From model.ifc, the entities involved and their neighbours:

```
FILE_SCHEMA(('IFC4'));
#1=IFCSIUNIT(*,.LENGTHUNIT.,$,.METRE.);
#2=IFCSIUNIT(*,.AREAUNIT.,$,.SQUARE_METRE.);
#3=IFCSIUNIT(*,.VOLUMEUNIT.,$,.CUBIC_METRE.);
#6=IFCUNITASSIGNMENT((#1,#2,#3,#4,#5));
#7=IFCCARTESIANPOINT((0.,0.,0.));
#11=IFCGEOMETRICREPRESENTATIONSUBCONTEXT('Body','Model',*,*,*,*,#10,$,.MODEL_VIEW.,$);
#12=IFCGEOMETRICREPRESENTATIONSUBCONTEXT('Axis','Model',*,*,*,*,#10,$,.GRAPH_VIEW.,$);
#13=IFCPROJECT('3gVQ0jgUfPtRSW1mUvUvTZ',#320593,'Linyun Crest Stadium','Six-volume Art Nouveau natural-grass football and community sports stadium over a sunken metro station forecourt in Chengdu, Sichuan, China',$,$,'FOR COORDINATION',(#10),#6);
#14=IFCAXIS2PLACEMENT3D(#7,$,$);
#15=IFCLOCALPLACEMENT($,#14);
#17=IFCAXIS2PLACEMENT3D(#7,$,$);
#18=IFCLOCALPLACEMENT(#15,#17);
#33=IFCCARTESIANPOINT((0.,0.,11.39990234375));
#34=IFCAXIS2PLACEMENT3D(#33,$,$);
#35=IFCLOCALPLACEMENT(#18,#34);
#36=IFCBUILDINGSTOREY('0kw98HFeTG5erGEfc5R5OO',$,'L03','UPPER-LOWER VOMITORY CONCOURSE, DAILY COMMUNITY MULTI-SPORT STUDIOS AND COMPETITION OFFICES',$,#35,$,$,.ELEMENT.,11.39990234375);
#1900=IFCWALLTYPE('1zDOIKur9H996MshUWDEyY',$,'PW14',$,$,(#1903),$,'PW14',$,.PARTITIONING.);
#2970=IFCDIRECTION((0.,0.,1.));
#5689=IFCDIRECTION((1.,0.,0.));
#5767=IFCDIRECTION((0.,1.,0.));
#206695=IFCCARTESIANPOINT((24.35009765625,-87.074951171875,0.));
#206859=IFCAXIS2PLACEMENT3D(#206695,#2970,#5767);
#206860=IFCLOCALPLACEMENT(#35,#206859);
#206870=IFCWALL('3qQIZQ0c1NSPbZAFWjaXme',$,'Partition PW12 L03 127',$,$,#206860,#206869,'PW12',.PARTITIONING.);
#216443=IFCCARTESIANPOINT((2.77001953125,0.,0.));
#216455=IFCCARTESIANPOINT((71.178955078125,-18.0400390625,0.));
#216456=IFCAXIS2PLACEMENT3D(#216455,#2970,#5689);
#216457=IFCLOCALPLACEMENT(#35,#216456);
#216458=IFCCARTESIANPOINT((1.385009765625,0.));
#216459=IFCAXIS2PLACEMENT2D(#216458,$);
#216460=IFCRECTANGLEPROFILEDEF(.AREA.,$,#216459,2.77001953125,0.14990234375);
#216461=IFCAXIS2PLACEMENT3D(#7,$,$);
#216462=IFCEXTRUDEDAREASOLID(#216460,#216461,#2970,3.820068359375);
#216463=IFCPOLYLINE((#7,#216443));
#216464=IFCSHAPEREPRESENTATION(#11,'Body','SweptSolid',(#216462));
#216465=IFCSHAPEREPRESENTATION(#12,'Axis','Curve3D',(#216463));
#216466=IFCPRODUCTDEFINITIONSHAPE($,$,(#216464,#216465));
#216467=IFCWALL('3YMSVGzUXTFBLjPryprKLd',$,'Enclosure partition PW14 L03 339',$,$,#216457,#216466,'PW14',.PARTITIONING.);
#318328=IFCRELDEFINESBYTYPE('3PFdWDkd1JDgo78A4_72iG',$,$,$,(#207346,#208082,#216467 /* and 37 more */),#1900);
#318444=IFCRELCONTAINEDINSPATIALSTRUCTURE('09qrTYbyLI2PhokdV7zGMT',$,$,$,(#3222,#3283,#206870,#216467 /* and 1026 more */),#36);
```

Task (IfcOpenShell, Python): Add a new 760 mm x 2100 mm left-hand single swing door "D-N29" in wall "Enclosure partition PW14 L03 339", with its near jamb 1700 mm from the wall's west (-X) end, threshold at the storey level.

```python
import numpy as np
import ifcopenshell
import ifcopenshell.api.feature
import ifcopenshell.api.geometry
import ifcopenshell.api.root
import ifcopenshell.api.spatial
import ifcopenshell.geom
import ifcopenshell.util.element
import ifcopenshell.util.placement
import ifcopenshell.util.representation
import ifcopenshell.util.shape
import ifcopenshell.util.unit

model = ifcopenshell.open("model.ifc")
unit_scale = ifcopenshell.util.unit.calculate_unit_scale(model)
settings = ifcopenshell.geom.settings()


def volume(element):
    """Net volume in cubic metres, openings subtracted."""
    shape = ifcopenshell.geom.create_shape(settings, element)
    return ifcopenshell.util.shape.get_volume(shape.geometry)


wall = model.by_guid("3YMSVGzUXTFBLjPryprKLd")
storey = ifcopenshell.util.element.get_container(wall, ifc_class="IfcBuildingStorey")
context = ifcopenshell.util.representation.get_context(model, "Model", "Body", "MODEL_VIEW")
before = volume(wall)

width, height, from_end, sill = 0.76, 2.1, 1.7, 0.0  # metres

# The wall runs along its own X axis, and the end named is its -X end.
wall_shape = ifcopenshell.geom.create_shape(settings, wall)
x, y, z = ifcopenshell.util.shape.get_vertices(wall_shape.geometry).T
start = x.min() + from_end
face, thickness = float(y.min()), float(y.max() - y.min())
wall_matrix = ifcopenshell.util.placement.get_local_placement(wall.ObjectPlacement)
level = ifcopenshell.util.placement.get_local_placement(storey.ObjectPlacement)[2, 3]


def in_wall(x, y):
    """Placement at x, y metres in the wall's axes, at sill height."""
    matrix = wall_matrix.copy()
    matrix[:, 3] = wall_matrix @ np.array([x / unit_scale, y / unit_scale, 0.0, 1.0])
    matrix[2, 3] = level + sill / unit_scale
    return matrix


# Opening: a box that overshoots both wall faces by 50 mm.
opening = ifcopenshell.api.root.create_entity(model, ifc_class="IfcOpeningElement", predefined_type="OPENING")
box = ifcopenshell.api.geometry.add_wall_representation(
    model, context=context, length=width, height=height, thickness=thickness + 0.1
)
ifcopenshell.api.geometry.assign_representation(model, product=opening, representation=box)
ifcopenshell.api.geometry.edit_object_placement(model, product=opening, matrix=in_wall(start, face - 0.05), is_si=False)
ifcopenshell.api.feature.add_feature(model, feature=opening, element=wall)

door = ifcopenshell.api.root.create_entity(model, ifc_class="IfcDoor", name="D-N29", predefined_type="DOOR")
door.OverallWidth, door.OverallHeight = width / unit_scale, height / unit_scale
door.OperationType = "SINGLE_SWING_LEFT"
body = ifcopenshell.api.geometry.add_door_representation(
    model,
    context=context,
    overall_width=door.OverallWidth,
    overall_height=door.OverallHeight,
    operation_type="SINGLE_SWING_LEFT",
    lining_properties={"LiningDepth": thickness / unit_scale, "ThresholdDepth": thickness / unit_scale},
)
ifcopenshell.api.geometry.assign_representation(model, product=door, representation=body)
ifcopenshell.api.spatial.assign_container(model, products=[door], relating_structure=storey)
ifcopenshell.api.feature.add_filling(model, opening=opening, element=door)

# The lining spans the wall, so the door starts at the wall face.
ifcopenshell.api.geometry.edit_object_placement(model, product=door, matrix=in_wall(start, face), is_si=False)

after = volume(wall)

print(f"wall volume {before:.3f} -> {after:.3f} m3")

model.write("model_updated.ifc")
```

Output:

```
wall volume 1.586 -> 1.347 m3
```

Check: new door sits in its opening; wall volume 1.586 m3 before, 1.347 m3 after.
